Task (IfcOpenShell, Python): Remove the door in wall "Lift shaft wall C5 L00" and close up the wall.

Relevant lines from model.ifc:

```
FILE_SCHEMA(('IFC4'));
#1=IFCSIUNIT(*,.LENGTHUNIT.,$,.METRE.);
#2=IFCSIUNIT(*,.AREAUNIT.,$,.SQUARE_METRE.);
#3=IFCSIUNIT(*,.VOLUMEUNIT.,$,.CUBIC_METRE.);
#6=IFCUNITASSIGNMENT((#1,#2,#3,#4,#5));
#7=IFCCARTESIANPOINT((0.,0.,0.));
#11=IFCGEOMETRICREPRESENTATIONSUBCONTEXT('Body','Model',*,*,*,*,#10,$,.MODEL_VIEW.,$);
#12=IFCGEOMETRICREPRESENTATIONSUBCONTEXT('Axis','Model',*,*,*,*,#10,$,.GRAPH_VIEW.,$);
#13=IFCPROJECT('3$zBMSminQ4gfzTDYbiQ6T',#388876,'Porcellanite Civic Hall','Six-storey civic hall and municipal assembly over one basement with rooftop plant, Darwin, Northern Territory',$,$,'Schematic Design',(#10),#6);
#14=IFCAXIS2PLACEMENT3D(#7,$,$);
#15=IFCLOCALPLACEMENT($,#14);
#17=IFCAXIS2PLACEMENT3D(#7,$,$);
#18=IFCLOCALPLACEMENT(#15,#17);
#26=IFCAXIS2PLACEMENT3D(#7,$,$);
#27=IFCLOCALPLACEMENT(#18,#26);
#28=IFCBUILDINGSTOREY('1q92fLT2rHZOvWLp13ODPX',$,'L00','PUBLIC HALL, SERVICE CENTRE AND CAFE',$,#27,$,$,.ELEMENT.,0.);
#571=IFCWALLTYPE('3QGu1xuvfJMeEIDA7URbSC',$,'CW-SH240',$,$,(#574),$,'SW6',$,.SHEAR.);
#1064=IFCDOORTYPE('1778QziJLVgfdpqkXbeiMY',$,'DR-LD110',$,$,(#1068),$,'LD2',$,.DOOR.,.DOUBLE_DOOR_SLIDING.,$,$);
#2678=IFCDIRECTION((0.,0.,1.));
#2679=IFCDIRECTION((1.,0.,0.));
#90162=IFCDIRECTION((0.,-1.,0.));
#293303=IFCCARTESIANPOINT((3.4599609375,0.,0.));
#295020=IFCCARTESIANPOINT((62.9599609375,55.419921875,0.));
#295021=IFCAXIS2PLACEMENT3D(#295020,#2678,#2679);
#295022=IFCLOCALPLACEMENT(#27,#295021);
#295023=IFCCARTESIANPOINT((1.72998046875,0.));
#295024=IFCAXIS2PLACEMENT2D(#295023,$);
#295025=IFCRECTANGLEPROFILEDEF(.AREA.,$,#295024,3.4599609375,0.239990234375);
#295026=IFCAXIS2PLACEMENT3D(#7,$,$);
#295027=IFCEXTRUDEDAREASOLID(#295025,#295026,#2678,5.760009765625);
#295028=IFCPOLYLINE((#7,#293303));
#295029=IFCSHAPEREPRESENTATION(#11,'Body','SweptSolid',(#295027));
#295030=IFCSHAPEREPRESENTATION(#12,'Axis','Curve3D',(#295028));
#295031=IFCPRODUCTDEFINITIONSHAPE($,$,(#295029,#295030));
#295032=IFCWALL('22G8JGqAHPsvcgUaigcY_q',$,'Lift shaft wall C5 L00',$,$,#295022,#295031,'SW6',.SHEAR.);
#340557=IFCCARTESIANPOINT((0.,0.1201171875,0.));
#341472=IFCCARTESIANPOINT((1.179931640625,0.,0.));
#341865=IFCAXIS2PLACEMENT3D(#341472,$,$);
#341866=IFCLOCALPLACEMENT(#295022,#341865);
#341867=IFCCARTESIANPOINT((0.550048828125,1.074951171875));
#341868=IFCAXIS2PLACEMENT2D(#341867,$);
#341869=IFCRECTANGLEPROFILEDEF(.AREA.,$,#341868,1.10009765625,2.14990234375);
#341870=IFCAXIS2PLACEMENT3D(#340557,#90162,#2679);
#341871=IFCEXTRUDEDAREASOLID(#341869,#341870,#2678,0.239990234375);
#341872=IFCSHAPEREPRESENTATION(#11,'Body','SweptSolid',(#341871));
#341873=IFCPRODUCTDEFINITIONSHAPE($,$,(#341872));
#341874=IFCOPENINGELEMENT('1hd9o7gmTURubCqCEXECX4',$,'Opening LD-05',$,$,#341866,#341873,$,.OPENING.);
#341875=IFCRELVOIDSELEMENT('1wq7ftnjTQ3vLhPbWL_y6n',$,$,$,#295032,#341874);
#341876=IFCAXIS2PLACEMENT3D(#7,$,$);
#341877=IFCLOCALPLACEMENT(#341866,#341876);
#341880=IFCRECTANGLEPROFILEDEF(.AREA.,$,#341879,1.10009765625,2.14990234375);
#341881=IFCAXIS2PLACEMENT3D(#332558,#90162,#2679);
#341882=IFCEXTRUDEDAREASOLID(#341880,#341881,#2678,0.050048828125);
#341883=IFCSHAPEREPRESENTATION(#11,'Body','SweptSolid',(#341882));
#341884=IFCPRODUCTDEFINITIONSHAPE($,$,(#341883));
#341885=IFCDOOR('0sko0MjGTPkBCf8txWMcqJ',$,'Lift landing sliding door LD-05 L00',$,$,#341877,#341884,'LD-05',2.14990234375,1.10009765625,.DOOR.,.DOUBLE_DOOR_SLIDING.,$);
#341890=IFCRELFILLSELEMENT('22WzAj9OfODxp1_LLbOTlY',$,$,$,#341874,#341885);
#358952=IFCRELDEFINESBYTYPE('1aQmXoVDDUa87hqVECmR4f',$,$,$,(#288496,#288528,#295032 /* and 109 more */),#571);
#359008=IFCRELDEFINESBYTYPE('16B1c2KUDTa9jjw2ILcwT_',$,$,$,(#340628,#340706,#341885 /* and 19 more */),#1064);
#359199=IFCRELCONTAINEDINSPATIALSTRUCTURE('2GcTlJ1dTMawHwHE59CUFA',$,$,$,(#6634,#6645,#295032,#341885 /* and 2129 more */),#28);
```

```python
import ifcopenshell
import ifcopenshell.api.feature
import ifcopenshell.api.root
import ifcopenshell.geom
import ifcopenshell.util.shape

model = ifcopenshell.open("model.ifc")
settings = ifcopenshell.geom.settings()


def volume(element):
    """Net volume in cubic metres, openings subtracted."""
    shape = ifcopenshell.geom.create_shape(settings, element)
    return ifcopenshell.util.shape.get_volume(shape.geometry)


door = model.by_guid("0sko0MjGTPkBCf8txWMcqJ")
opening = door.FillsVoids[0].RelatingOpeningElement
wall = opening.VoidsElements[0].RelatingBuildingElement
before = volume(wall)

ifcopenshell.api.root.remove_product(model, product=door)
ifcopenshell.api.feature.remove_feature(model, feature=opening)

after = volume(wall)

print(f"wall volume {before:.3f} -> {after:.3f} m3")

model.write("model-out.ifc")
```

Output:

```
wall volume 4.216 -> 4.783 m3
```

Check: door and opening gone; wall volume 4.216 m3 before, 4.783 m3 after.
